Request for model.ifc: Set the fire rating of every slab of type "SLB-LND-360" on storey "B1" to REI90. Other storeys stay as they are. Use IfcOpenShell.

First a look at what the model holds.

```python
import ifcopenshell
import ifcopenshell.util.element

model = ifcopenshell.open("model.ifc")
print(model.schema)
storey = next(s for s in model.by_type("IfcBuildingStorey") if s.Name == "B1")
slabs = [e for e in ifcopenshell.util.element.get_decomposition(storey) if e.is_a("IfcSlab")]
seen = {}
for e in slabs:
    element_type = ifcopenshell.util.element.get_type(e)
    key = (element_type.Name if element_type != e and element_type else None, ifcopenshell.util.element.get_pset(e, "Pset_SlabCommon", "FireRating"))
    seen[key] = seen.get(key, 0) + 1
for (name, value), count in sorted(seen.items(), key=str):
    print(count, "x", name, "|", value)
```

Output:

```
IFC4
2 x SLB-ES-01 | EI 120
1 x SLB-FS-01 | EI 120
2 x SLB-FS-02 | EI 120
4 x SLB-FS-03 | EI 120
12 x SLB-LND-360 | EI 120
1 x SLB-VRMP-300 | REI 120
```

```python
import ifcopenshell
import ifcopenshell.api.pset
import ifcopenshell.util.element

model = ifcopenshell.open("model.ifc")

storey = next(s for s in model.by_type("IfcBuildingStorey") if s.Name == "B1")
slabs = [e for e in ifcopenshell.util.element.get_decomposition(storey) if e.is_a("IfcSlab")]

count = 0
for e in slabs:
    element_type = ifcopenshell.util.element.get_type(e)
    if element_type in (None, e) or element_type.Name != "SLB-LND-360":
        continue
    # add_pset returns the element's existing set when there is one.
    pset = ifcopenshell.api.pset.add_pset(model, product=e, name="Pset_SlabCommon")
    ifcopenshell.api.pset.edit_pset(model, pset=pset, properties={"FireRating": "REI90"})
    count += 1

print(count, "slabs updated")

model.write("model_edited.ifc")
```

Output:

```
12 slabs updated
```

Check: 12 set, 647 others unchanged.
